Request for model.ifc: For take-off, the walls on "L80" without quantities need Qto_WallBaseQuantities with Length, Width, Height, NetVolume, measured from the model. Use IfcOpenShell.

First a look at what the model holds.

```python
import ifcopenshell
import ifcopenshell.util.element
import ifcopenshell.util.unit

model = ifcopenshell.open("model.ifc")
print(model.schema)
for unit_type in ("LENGTHUNIT", "AREAUNIT", "VOLUMEUNIT"):
    print(unit_type, ifcopenshell.util.unit.calculate_unit_scale(model, unit_type))
storey = next(s for s in model.by_type("IfcBuildingStorey") if s.Name == "L80")
walls = [e for e in ifcopenshell.util.element.get_decomposition(storey) if e.is_a("IfcWall")]
for e in sorted(walls, key=lambda e: e.id()):
    print(e.id(), e.is_a(), e.Name, list(ifcopenshell.util.element.get_psets(e, qtos_only=True)), sep=" | ")
```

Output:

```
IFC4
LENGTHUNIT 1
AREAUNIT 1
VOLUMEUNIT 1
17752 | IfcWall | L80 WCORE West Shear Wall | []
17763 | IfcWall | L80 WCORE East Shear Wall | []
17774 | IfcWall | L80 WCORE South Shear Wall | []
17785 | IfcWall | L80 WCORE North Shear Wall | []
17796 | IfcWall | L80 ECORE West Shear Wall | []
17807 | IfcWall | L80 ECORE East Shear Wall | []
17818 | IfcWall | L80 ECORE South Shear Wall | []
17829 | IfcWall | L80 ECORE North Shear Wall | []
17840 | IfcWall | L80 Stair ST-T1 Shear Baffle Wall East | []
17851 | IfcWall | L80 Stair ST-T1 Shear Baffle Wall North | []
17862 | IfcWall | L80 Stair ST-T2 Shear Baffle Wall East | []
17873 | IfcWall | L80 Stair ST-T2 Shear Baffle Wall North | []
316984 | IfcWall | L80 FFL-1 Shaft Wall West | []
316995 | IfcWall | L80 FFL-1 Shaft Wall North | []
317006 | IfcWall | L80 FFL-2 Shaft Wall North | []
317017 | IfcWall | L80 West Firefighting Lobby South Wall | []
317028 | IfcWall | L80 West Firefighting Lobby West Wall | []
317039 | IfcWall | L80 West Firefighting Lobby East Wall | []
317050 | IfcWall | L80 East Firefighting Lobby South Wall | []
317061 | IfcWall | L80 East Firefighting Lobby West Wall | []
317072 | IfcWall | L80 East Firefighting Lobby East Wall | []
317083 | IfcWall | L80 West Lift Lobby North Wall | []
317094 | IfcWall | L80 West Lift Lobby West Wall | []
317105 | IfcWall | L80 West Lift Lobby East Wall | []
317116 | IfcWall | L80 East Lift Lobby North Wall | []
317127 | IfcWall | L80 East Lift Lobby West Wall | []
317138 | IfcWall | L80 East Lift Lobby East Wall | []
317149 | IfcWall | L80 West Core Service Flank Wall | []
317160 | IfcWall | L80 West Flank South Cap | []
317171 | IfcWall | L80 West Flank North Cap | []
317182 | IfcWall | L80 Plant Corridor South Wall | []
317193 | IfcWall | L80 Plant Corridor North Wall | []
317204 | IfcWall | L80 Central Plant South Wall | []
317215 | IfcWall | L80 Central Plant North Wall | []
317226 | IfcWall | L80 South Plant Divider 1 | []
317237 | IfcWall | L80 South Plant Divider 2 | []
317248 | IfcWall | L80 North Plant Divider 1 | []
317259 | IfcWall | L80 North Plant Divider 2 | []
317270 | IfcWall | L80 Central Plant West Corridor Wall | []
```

```python
import ifcopenshell
import ifcopenshell.api.pset
import ifcopenshell.geom
import ifcopenshell.util.element
import ifcopenshell.util.shape
import ifcopenshell.util.unit

model = ifcopenshell.open("model.ifc")
unit_scale = ifcopenshell.util.unit.calculate_unit_scale(model)
volume_scale = ifcopenshell.util.unit.calculate_unit_scale(model, "VOLUMEUNIT")
settings = ifcopenshell.geom.settings()

storey = next(s for s in model.by_type("IfcBuildingStorey") if s.Name == "L80")
walls = [e for e in ifcopenshell.util.element.get_decomposition(storey) if e.is_a("IfcWall")]

for e in sorted(walls, key=lambda e: e.id()):
    if ifcopenshell.util.element.get_psets(e, qtos_only=True, should_inherit=False):
        continue
    # Geometry comes back in metres, in the element's own axes.
    shape = ifcopenshell.geom.create_shape(settings, e)
    values = {
        "Length": ifcopenshell.util.shape.get_x(shape.geometry) / unit_scale,
        "Width": ifcopenshell.util.shape.get_y(shape.geometry) / unit_scale,
        "Height": ifcopenshell.util.shape.get_z(shape.geometry) / unit_scale,
        "NetVolume": ifcopenshell.util.shape.get_volume(shape.geometry) / volume_scale,
    }
    qto = ifcopenshell.api.pset.add_qto(model, product=e, name="Qto_WallBaseQuantities")
    ifcopenshell.api.pset.edit_qto(model, qto=qto, properties=values)
    print(e.id(), {k: round(v, 3) for k, v in values.items()})

model.write("model-out.ifc")
```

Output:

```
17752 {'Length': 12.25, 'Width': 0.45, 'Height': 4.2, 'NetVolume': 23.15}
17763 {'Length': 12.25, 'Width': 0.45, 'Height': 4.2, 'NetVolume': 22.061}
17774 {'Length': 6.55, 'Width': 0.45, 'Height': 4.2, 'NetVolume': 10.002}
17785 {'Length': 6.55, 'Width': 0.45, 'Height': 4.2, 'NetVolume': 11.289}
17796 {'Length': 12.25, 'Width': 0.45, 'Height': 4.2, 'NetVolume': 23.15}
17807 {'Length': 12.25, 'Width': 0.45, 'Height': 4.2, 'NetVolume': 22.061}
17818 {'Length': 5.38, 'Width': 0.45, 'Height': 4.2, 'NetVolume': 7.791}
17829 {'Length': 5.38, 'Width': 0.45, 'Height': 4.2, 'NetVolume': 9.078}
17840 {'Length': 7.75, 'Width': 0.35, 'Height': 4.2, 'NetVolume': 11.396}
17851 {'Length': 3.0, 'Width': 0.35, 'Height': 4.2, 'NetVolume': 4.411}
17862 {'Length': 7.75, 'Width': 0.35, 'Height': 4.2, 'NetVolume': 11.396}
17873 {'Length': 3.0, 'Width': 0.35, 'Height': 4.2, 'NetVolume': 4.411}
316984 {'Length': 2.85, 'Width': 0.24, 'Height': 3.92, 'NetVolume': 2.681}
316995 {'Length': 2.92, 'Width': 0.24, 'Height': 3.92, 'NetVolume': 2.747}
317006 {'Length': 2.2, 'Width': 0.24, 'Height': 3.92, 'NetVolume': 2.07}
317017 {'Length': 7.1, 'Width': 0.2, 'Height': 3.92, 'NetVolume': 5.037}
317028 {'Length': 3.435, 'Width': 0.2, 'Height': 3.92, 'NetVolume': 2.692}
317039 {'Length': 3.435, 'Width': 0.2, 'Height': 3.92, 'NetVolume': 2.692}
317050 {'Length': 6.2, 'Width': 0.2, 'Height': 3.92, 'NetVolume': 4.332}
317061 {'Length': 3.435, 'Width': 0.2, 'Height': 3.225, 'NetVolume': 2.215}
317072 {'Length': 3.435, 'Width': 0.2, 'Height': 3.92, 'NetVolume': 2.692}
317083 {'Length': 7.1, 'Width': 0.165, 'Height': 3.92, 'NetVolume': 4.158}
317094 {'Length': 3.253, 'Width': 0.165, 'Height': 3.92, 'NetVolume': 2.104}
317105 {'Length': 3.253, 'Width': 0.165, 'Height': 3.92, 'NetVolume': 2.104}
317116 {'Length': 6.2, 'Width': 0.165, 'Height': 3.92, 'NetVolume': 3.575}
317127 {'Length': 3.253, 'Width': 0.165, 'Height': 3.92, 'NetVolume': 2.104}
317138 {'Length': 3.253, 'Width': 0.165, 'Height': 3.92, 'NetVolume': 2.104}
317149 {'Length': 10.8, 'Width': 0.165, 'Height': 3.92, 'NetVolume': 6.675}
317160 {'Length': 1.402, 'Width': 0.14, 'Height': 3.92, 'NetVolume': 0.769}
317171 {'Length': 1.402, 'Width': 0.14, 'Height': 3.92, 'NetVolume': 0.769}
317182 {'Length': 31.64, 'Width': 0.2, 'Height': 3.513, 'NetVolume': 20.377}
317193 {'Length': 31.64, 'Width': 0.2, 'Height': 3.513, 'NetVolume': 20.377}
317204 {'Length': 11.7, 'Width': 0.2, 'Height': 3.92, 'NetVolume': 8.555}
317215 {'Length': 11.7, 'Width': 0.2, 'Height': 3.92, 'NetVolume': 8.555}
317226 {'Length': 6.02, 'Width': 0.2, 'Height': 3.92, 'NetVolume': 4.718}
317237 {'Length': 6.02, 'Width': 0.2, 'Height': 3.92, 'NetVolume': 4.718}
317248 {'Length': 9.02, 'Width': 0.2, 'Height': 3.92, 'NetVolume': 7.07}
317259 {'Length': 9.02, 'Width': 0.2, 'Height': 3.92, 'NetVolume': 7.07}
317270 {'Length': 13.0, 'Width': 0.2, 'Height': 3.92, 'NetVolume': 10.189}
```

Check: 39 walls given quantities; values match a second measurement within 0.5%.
